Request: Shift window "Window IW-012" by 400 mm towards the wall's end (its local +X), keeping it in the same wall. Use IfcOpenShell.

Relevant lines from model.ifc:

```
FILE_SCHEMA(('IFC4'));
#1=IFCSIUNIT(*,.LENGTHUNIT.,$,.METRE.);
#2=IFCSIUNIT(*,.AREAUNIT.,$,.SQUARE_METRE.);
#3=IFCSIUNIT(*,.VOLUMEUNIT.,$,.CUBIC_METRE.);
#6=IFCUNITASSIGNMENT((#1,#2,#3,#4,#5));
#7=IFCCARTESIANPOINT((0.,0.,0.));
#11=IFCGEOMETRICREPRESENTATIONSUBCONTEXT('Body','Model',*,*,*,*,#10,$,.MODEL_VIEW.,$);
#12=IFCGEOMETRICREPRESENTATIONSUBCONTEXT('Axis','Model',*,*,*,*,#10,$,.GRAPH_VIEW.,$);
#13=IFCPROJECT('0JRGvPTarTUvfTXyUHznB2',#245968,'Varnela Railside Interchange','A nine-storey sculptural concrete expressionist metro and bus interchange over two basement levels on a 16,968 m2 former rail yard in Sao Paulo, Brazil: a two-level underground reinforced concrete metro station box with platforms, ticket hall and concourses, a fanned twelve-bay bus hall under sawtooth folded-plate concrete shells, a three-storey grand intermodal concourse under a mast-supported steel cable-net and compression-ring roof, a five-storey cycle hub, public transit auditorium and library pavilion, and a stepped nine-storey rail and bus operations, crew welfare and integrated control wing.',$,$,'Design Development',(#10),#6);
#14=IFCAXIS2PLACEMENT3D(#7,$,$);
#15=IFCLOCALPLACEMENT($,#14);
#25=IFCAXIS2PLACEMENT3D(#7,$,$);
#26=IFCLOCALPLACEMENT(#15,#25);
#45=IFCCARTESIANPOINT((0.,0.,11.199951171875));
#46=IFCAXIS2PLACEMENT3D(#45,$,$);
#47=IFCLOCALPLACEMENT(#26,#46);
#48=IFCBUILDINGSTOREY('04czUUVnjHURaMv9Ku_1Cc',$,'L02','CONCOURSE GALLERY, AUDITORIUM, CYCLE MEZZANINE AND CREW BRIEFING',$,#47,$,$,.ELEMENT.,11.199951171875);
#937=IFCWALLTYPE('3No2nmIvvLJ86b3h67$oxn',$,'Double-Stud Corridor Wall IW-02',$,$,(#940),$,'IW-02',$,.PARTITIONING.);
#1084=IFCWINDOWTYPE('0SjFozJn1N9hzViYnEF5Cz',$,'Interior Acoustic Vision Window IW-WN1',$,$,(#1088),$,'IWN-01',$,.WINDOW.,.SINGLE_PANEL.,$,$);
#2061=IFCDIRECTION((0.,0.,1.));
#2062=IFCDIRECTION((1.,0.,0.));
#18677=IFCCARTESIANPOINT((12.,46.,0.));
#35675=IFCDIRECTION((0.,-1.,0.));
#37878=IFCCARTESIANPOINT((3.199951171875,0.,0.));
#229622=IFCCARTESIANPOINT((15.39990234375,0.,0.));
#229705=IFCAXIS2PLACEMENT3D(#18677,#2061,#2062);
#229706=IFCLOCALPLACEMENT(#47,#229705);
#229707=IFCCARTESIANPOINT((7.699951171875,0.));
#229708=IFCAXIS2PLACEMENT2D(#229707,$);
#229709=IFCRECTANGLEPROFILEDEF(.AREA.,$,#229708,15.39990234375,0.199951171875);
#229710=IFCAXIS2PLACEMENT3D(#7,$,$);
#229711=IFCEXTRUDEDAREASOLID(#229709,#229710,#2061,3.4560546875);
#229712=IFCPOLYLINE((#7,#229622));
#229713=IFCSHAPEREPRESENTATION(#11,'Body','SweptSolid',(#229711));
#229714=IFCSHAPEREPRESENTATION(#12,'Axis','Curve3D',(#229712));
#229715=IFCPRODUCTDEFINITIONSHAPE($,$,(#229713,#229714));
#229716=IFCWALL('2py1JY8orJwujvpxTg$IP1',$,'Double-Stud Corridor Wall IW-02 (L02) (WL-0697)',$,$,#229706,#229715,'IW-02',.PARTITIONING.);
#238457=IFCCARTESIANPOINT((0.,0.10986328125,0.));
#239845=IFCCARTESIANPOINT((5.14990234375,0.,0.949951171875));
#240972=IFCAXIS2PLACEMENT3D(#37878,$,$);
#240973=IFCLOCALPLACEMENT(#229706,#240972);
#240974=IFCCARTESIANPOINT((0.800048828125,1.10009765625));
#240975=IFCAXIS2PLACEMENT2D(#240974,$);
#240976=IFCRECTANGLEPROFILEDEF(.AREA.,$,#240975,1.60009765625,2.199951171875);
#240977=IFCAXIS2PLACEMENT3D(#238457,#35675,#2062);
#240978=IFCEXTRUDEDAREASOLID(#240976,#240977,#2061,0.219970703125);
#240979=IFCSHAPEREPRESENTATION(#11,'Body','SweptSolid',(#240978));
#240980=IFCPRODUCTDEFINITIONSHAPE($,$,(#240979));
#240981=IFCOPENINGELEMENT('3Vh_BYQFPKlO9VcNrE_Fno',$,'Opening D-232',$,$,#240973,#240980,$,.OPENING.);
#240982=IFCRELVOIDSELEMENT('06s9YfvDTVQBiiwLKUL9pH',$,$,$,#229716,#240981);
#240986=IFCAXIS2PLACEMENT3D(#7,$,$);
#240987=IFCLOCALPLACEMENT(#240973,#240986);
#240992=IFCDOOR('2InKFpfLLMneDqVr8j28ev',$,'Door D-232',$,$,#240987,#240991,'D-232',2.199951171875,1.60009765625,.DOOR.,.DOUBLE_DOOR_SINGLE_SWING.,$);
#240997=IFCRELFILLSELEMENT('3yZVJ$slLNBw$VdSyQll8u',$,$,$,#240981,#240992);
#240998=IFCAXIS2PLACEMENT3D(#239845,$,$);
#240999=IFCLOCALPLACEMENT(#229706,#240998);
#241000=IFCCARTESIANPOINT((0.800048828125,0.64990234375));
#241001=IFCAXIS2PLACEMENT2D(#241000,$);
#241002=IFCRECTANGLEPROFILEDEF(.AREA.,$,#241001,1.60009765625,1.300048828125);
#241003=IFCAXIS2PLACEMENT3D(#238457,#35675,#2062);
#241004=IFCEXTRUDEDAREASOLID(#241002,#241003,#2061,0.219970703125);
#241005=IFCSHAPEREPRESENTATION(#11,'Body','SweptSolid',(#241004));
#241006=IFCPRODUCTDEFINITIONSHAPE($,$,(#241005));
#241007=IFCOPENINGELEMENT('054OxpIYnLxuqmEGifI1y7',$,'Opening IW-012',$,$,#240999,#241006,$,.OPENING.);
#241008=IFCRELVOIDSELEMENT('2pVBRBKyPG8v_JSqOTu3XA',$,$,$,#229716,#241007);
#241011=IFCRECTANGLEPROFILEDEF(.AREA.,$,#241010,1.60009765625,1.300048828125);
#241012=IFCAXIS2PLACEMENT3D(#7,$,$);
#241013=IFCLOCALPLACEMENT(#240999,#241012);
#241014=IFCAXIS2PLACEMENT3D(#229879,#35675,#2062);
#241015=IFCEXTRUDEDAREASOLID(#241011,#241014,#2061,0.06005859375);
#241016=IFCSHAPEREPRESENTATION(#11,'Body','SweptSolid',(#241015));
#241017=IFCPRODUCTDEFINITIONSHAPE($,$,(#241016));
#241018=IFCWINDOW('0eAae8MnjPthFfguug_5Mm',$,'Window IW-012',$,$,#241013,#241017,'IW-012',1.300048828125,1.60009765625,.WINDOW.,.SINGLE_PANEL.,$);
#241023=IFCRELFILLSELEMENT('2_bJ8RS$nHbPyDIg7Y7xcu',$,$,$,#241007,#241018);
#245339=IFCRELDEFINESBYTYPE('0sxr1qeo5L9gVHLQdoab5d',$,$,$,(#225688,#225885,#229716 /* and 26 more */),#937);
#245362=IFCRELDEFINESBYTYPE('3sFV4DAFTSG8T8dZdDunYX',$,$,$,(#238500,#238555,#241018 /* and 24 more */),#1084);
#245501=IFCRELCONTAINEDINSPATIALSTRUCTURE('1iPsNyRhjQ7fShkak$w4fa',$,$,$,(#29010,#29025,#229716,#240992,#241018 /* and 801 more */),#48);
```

```python
import ifcopenshell
import ifcopenshell.api.geometry
import ifcopenshell.util.placement
import ifcopenshell.util.unit

model = ifcopenshell.open("model.ifc")
unit_scale = ifcopenshell.util.unit.calculate_unit_scale(model)

window = model.by_guid("0eAae8MnjPthFfguug_5Mm")
opening = window.FillsVoids[0].RelatingOpeningElement
wall = opening.VoidsElements[0].RelatingBuildingElement

wall_matrix = ifcopenshell.util.placement.get_local_placement(wall.ObjectPlacement)
shift = wall_matrix[:3, 0] * 0.4 / unit_scale
before = ifcopenshell.util.placement.get_local_placement(window.ObjectPlacement)[:3, 3].copy()

# The window is placed relative to its opening, so it follows when the opening moves.
matrix = ifcopenshell.util.placement.get_local_placement(opening.ObjectPlacement)
matrix[:3, 3] += shift
ifcopenshell.api.geometry.edit_object_placement(
    model, product=opening, matrix=matrix, is_si=False, should_transform_children=True
)

after = ifcopenshell.util.placement.get_local_placement(window.ObjectPlacement)[:3, 3]
print("window moved by", (after - before).round(3) + 0.0)

model.write("model-out.ifc")
```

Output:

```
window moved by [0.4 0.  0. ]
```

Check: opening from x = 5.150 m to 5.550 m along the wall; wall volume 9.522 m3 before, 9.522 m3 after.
